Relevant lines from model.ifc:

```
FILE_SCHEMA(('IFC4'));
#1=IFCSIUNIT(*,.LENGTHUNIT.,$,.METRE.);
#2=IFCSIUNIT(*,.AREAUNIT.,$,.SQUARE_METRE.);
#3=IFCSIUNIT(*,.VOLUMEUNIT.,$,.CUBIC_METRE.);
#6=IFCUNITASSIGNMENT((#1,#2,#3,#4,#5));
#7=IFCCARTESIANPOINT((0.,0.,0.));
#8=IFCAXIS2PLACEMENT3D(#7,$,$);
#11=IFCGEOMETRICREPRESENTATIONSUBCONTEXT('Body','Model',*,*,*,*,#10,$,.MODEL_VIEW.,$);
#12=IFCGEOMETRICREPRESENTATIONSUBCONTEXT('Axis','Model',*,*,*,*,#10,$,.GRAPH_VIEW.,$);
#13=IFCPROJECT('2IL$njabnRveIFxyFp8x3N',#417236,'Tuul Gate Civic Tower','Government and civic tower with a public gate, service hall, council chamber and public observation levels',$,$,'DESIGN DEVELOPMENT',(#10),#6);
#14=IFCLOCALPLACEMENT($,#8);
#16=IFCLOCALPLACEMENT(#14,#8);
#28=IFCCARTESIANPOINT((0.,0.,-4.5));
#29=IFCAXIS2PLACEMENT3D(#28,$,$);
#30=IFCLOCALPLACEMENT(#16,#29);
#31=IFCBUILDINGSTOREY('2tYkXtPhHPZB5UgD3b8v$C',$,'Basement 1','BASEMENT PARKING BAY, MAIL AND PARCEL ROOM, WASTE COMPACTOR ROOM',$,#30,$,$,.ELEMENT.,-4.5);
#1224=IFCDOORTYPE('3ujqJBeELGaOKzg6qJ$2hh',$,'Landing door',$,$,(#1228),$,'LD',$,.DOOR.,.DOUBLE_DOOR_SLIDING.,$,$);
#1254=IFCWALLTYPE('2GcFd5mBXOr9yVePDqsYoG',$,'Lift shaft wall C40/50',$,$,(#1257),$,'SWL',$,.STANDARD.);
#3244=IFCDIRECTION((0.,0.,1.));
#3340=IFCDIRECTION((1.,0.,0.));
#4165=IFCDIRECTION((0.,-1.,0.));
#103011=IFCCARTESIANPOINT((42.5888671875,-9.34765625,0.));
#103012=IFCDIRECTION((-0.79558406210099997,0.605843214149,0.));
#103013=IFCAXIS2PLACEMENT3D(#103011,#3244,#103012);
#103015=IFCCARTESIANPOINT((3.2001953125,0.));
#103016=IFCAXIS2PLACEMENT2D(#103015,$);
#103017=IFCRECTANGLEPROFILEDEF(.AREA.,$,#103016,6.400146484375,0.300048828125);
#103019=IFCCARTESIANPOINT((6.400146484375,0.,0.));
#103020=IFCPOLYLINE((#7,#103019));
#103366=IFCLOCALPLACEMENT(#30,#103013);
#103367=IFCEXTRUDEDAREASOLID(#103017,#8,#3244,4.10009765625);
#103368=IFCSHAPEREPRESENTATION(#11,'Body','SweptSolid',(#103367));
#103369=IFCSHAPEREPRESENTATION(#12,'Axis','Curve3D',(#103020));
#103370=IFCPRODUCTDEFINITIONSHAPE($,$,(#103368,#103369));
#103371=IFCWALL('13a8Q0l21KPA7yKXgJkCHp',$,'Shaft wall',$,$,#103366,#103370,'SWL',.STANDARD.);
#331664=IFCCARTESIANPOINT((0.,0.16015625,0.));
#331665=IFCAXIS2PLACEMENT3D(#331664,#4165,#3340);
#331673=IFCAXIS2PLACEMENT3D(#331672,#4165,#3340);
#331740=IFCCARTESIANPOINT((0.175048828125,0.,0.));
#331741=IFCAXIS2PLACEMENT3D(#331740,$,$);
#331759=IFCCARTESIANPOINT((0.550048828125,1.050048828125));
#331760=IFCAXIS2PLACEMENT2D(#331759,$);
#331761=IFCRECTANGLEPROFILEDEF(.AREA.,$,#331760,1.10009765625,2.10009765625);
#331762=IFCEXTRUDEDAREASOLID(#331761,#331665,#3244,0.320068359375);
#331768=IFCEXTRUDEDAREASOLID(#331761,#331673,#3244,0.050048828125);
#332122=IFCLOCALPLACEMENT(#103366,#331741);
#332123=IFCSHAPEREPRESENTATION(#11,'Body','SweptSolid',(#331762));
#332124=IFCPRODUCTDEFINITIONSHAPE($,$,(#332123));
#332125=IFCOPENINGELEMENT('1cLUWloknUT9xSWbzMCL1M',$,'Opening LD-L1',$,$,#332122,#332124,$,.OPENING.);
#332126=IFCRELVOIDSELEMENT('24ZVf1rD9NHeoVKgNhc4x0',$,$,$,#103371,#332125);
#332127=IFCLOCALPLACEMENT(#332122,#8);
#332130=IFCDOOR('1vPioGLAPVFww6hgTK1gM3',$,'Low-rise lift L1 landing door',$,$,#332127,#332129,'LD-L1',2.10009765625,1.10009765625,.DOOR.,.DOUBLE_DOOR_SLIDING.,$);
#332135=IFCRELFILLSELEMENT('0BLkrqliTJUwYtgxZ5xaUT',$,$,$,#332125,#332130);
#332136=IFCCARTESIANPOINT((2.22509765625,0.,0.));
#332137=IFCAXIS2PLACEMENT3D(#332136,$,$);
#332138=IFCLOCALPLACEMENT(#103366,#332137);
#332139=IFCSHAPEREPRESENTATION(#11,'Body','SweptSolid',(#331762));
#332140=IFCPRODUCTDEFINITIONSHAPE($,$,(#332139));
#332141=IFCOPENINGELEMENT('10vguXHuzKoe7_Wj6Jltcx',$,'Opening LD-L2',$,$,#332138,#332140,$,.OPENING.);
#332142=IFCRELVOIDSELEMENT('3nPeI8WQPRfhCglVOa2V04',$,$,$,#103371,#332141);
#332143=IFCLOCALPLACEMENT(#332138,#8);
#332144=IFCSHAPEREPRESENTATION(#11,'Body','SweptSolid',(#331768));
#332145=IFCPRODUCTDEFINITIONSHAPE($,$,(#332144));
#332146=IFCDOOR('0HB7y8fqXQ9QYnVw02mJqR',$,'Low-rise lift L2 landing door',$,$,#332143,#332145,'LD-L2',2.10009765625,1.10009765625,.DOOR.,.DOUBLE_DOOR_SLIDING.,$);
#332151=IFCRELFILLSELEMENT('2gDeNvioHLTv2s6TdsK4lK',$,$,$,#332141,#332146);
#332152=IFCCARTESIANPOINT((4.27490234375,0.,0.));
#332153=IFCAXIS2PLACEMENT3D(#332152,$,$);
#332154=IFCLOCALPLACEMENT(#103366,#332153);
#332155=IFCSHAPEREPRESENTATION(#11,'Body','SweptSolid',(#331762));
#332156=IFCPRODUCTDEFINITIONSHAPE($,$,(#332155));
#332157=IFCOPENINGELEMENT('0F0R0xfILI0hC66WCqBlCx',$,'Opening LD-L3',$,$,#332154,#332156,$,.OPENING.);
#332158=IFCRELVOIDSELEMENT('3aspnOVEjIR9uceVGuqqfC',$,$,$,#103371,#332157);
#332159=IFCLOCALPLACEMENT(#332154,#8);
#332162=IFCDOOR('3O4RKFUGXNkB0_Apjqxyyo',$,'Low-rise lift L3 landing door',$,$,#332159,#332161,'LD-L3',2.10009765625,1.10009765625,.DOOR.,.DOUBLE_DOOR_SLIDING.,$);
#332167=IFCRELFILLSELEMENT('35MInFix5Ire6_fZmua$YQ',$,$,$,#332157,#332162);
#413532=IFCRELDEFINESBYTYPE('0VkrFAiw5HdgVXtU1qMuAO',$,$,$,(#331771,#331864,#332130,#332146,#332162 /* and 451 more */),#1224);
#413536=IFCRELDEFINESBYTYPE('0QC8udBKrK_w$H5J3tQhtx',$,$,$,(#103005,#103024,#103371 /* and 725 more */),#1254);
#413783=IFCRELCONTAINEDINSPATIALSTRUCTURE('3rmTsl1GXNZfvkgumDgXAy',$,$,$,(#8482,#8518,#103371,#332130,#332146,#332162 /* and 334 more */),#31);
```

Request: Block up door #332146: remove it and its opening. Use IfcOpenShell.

```python
import ifcopenshell
import ifcopenshell.api.feature
import ifcopenshell.api.root
import ifcopenshell.geom
import ifcopenshell.util.shape

model = ifcopenshell.open("model.ifc")
settings = ifcopenshell.geom.settings()


def volume(element):
    """Net volume in cubic metres, openings subtracted."""
    shape = ifcopenshell.geom.create_shape(settings, element)
    return ifcopenshell.util.shape.get_volume(shape.geometry)


door = model.by_guid("0HB7y8fqXQ9QYnVw02mJqR")
opening = door.FillsVoids[0].RelatingOpeningElement
wall = opening.VoidsElements[0].RelatingBuildingElement
before = volume(wall)

ifcopenshell.api.root.remove_product(model, product=door)
ifcopenshell.api.feature.remove_feature(model, feature=opening)

after = volume(wall)

print(f"wall volume {before:.3f} -> {after:.3f} m3")

model.write("model_edited.ifc")
```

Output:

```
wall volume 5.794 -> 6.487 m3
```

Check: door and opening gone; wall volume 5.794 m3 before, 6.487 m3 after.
